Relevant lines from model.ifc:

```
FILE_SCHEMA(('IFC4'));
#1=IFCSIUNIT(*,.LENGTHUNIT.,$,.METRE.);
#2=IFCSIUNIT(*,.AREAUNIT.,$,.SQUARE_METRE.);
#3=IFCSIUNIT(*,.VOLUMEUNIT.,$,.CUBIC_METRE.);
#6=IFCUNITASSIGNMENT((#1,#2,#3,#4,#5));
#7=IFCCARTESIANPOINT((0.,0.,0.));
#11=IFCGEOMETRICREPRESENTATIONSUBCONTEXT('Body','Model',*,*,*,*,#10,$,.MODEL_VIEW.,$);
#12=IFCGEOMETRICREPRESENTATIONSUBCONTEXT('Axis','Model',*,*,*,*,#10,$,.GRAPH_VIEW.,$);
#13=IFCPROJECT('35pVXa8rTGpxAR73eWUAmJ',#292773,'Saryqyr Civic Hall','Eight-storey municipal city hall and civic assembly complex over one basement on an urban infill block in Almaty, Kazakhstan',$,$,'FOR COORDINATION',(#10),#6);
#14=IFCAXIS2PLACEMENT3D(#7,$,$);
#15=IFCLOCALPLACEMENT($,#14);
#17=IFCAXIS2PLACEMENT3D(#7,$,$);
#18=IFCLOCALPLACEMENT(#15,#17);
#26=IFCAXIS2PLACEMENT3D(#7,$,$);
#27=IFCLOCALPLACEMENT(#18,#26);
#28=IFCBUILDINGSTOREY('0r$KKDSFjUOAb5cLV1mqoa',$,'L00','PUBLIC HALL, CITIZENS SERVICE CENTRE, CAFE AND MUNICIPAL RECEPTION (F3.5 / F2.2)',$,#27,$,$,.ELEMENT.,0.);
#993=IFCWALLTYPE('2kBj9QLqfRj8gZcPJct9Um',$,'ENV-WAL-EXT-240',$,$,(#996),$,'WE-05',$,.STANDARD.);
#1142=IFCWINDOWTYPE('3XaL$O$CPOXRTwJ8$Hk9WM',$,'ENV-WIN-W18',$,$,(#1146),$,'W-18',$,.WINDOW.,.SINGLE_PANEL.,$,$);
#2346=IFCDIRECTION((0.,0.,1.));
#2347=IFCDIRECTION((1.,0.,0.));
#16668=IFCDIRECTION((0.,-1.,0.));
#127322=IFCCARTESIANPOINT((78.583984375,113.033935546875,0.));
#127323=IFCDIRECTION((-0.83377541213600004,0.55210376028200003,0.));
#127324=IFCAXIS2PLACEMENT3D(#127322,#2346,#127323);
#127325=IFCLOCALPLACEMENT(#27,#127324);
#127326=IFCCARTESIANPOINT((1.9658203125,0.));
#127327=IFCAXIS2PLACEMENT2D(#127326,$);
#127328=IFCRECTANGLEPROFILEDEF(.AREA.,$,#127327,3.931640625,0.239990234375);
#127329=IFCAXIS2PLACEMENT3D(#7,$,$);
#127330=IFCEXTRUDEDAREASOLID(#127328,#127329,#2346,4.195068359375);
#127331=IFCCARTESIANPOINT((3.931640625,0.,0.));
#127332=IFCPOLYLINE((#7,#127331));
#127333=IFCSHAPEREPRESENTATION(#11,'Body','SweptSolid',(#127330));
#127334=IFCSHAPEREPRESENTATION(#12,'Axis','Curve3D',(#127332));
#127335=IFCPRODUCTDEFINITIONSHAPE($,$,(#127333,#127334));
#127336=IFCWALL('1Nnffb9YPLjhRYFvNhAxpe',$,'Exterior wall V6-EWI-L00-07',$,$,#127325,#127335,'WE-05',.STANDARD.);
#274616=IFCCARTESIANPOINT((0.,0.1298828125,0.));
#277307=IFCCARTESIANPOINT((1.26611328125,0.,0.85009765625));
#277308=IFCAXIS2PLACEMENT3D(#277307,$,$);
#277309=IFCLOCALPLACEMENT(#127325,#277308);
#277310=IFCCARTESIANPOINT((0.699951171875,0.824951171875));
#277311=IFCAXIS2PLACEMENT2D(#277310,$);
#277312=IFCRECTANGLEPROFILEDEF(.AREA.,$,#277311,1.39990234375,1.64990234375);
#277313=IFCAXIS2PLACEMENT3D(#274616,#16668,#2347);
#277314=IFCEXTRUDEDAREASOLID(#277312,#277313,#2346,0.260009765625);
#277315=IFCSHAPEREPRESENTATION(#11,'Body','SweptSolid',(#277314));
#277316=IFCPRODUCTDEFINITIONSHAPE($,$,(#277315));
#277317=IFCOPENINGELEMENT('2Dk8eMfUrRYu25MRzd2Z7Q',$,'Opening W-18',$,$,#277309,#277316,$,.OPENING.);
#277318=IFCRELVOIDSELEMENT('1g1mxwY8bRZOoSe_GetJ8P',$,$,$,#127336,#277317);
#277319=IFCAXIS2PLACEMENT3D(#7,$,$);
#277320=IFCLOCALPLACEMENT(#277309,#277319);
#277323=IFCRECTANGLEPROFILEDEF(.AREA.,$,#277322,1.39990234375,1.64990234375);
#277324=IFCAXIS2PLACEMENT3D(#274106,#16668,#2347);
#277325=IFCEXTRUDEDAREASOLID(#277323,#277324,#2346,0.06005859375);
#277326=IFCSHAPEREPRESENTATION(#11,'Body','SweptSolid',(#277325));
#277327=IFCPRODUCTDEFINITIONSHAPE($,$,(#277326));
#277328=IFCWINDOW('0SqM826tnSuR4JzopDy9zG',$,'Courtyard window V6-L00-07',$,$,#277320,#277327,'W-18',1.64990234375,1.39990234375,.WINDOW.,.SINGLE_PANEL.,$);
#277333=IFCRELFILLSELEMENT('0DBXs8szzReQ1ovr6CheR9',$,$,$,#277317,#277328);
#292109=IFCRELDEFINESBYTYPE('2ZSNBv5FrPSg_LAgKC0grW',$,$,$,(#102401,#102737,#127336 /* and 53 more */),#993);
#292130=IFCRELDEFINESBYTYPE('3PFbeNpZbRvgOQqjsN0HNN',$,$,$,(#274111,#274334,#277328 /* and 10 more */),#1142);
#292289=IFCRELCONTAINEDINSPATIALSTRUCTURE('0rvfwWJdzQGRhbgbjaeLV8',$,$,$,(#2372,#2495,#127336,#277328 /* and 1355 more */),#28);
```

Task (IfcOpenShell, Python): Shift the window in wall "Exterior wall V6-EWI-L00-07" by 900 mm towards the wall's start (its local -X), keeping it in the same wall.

```python
import ifcopenshell
import ifcopenshell.api.geometry
import ifcopenshell.util.placement
import ifcopenshell.util.unit

model = ifcopenshell.open("model.ifc")
unit_scale = ifcopenshell.util.unit.calculate_unit_scale(model)

window = model.by_id(277328)
opening = window.FillsVoids[0].RelatingOpeningElement
wall = opening.VoidsElements[0].RelatingBuildingElement

wall_matrix = ifcopenshell.util.placement.get_local_placement(wall.ObjectPlacement)
shift = wall_matrix[:3, 0] * -0.9 / unit_scale
before = ifcopenshell.util.placement.get_local_placement(window.ObjectPlacement)[:3, 3].copy()

# The window is placed relative to its opening, so it follows when the opening moves.
matrix = ifcopenshell.util.placement.get_local_placement(opening.ObjectPlacement)
matrix[:3, 3] += shift
ifcopenshell.api.geometry.edit_object_placement(
    model, product=opening, matrix=matrix, is_si=False, should_transform_children=True
)

after = ifcopenshell.util.placement.get_local_placement(window.ObjectPlacement)[:3, 3]
print("window moved by", (after - before).round(3) + 0.0)

model.write("model_edited.ifc")
```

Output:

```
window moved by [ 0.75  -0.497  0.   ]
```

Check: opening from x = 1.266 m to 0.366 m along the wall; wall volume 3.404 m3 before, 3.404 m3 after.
